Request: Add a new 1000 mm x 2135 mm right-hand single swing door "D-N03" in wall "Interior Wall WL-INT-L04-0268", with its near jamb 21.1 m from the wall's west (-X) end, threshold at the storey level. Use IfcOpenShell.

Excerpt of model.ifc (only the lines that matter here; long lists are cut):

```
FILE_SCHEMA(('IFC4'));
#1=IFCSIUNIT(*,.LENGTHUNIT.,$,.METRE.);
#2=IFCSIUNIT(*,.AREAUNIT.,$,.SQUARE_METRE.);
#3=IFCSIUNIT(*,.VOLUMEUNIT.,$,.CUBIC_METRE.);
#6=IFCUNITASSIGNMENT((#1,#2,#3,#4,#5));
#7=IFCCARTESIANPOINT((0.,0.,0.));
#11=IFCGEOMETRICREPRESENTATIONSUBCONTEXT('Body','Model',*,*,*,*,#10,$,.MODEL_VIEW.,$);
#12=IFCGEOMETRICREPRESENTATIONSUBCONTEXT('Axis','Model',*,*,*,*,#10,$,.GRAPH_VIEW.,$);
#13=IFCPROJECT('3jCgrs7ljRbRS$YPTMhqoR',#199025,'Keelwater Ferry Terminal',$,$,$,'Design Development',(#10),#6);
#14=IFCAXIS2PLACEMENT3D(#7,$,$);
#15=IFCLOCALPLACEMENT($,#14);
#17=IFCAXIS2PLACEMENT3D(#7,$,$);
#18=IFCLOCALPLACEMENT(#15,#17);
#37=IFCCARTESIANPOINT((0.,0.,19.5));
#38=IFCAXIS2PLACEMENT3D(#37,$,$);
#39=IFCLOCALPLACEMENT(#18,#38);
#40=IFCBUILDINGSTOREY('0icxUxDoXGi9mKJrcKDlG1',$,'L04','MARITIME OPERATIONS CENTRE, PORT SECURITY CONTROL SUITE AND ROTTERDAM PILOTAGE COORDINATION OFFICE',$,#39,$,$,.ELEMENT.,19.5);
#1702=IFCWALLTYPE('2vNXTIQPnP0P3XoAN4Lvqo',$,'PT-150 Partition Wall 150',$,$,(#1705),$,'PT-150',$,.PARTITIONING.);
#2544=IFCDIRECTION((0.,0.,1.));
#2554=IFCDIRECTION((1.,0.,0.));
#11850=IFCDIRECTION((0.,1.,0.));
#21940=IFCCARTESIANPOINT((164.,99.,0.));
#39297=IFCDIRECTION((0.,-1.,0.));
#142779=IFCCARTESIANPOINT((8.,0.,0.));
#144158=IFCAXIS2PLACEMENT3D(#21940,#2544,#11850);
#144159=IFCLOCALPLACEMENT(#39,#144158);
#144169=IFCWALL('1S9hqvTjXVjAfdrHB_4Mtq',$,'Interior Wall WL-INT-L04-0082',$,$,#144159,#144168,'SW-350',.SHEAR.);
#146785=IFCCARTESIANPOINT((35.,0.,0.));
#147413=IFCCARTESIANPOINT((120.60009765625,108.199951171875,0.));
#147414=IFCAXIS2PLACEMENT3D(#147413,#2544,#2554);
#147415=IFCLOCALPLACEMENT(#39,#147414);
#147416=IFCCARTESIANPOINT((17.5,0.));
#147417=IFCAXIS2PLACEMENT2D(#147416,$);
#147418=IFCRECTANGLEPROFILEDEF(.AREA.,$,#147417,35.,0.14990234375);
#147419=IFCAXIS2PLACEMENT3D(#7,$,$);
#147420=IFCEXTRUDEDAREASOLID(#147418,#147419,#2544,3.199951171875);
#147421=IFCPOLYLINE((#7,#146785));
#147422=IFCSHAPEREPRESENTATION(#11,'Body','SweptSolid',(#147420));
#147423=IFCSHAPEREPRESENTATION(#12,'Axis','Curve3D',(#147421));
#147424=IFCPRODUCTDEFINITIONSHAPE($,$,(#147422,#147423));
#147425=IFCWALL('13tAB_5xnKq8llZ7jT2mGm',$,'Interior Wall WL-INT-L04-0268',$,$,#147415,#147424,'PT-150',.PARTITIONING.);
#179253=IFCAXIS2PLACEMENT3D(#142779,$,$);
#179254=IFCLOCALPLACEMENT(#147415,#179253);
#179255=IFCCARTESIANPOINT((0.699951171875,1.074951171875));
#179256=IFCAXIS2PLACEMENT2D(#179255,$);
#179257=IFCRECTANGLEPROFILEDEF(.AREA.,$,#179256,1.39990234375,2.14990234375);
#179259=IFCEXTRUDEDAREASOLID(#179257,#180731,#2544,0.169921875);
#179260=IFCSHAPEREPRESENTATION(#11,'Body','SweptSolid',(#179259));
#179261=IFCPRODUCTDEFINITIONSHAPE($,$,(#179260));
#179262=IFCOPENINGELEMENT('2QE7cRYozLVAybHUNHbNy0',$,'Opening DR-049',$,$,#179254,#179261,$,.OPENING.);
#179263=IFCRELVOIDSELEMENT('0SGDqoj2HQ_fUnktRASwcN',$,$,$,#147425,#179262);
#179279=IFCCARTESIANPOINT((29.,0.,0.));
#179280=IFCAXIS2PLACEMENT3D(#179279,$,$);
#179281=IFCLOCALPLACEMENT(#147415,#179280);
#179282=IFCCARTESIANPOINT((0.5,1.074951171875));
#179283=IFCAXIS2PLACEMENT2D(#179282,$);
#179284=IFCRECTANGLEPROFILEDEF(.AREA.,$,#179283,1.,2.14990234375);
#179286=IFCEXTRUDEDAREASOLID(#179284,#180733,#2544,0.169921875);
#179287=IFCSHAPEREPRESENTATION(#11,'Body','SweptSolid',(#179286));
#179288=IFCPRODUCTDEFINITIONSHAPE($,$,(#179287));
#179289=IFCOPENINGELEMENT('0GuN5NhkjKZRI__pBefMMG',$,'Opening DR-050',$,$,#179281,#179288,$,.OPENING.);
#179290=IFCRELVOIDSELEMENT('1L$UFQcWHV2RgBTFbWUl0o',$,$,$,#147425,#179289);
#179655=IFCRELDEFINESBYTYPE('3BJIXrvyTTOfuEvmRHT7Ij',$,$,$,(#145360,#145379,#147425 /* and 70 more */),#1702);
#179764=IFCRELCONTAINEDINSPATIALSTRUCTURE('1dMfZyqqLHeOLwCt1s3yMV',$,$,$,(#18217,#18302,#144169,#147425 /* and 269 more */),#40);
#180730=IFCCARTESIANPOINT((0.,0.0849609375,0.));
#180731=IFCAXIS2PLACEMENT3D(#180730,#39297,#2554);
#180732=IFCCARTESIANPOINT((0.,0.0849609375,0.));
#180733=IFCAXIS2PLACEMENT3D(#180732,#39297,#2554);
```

```python
import numpy as np
import ifcopenshell
import ifcopenshell.api.feature
import ifcopenshell.api.geometry
import ifcopenshell.api.root
import ifcopenshell.api.spatial
import ifcopenshell.geom
import ifcopenshell.util.element
import ifcopenshell.util.placement
import ifcopenshell.util.representation
import ifcopenshell.util.shape
import ifcopenshell.util.unit

model = ifcopenshell.open("model.ifc")
unit_scale = ifcopenshell.util.unit.calculate_unit_scale(model)
settings = ifcopenshell.geom.settings()


def volume(element):
    """Net volume in cubic metres, openings subtracted."""
    shape = ifcopenshell.geom.create_shape(settings, element)
    return ifcopenshell.util.shape.get_volume(shape.geometry)


wall = model.by_id(147425)
storey = ifcopenshell.util.element.get_container(wall, ifc_class="IfcBuildingStorey")
context = ifcopenshell.util.representation.get_context(model, "Model", "Body", "MODEL_VIEW")
before = volume(wall)

width, height, from_end, sill = 1, 2.135, 21.1, 0.0  # metres

# The wall runs along its own X axis, and the end named is its -X end.
wall_shape = ifcopenshell.geom.create_shape(settings, wall)
x, y, z = ifcopenshell.util.shape.get_vertices(wall_shape.geometry).T
start = x.min() + from_end
face, thickness = float(y.min()), float(y.max() - y.min())
wall_matrix = ifcopenshell.util.placement.get_local_placement(wall.ObjectPlacement)
level = ifcopenshell.util.placement.get_local_placement(storey.ObjectPlacement)[2, 3]


def in_wall(x, y):
    """Placement at x, y metres in the wall's axes, at sill height."""
    matrix = wall_matrix.copy()
    matrix[:, 3] = wall_matrix @ np.array([x / unit_scale, y / unit_scale, 0.0, 1.0])
    matrix[2, 3] = level + sill / unit_scale
    return matrix


# Opening: a box that overshoots both wall faces by 50 mm.
opening = ifcopenshell.api.root.create_entity(model, ifc_class="IfcOpeningElement", predefined_type="OPENING")
box = ifcopenshell.api.geometry.add_wall_representation(
    model, context=context, length=width, height=height, thickness=thickness + 0.1
)
ifcopenshell.api.geometry.assign_representation(model, product=opening, representation=box)
ifcopenshell.api.geometry.edit_object_placement(model, product=opening, matrix=in_wall(start, face - 0.05), is_si=False)
ifcopenshell.api.feature.add_feature(model, feature=opening, element=wall)

door = ifcopenshell.api.root.create_entity(model, ifc_class="IfcDoor", name="D-N03", predefined_type="DOOR")
door.OverallWidth, door.OverallHeight = width / unit_scale, height / unit_scale
door.OperationType = "SINGLE_SWING_RIGHT"
body = ifcopenshell.api.geometry.add_door_representation(
    model,
    context=context,
    overall_width=door.OverallWidth,
    overall_height=door.OverallHeight,
    operation_type="SINGLE_SWING_RIGHT",
    lining_properties={"LiningDepth": thickness / unit_scale, "ThresholdDepth": thickness / unit_scale},
)
ifcopenshell.api.geometry.assign_representation(model, product=door, representation=body)
ifcopenshell.api.spatial.assign_container(model, products=[door], relating_structure=storey)
ifcopenshell.api.feature.add_filling(model, opening=opening, element=door)

# The lining spans the wall, so the door starts at the wall face.
ifcopenshell.api.geometry.edit_object_placement(model, product=door, matrix=in_wall(start, face), is_si=False)

after = volume(wall)

print(f"wall volume {before:.3f} -> {after:.3f} m3")

model.write("model_updated.ifc")
```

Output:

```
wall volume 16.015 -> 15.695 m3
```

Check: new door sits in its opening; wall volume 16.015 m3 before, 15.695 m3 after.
